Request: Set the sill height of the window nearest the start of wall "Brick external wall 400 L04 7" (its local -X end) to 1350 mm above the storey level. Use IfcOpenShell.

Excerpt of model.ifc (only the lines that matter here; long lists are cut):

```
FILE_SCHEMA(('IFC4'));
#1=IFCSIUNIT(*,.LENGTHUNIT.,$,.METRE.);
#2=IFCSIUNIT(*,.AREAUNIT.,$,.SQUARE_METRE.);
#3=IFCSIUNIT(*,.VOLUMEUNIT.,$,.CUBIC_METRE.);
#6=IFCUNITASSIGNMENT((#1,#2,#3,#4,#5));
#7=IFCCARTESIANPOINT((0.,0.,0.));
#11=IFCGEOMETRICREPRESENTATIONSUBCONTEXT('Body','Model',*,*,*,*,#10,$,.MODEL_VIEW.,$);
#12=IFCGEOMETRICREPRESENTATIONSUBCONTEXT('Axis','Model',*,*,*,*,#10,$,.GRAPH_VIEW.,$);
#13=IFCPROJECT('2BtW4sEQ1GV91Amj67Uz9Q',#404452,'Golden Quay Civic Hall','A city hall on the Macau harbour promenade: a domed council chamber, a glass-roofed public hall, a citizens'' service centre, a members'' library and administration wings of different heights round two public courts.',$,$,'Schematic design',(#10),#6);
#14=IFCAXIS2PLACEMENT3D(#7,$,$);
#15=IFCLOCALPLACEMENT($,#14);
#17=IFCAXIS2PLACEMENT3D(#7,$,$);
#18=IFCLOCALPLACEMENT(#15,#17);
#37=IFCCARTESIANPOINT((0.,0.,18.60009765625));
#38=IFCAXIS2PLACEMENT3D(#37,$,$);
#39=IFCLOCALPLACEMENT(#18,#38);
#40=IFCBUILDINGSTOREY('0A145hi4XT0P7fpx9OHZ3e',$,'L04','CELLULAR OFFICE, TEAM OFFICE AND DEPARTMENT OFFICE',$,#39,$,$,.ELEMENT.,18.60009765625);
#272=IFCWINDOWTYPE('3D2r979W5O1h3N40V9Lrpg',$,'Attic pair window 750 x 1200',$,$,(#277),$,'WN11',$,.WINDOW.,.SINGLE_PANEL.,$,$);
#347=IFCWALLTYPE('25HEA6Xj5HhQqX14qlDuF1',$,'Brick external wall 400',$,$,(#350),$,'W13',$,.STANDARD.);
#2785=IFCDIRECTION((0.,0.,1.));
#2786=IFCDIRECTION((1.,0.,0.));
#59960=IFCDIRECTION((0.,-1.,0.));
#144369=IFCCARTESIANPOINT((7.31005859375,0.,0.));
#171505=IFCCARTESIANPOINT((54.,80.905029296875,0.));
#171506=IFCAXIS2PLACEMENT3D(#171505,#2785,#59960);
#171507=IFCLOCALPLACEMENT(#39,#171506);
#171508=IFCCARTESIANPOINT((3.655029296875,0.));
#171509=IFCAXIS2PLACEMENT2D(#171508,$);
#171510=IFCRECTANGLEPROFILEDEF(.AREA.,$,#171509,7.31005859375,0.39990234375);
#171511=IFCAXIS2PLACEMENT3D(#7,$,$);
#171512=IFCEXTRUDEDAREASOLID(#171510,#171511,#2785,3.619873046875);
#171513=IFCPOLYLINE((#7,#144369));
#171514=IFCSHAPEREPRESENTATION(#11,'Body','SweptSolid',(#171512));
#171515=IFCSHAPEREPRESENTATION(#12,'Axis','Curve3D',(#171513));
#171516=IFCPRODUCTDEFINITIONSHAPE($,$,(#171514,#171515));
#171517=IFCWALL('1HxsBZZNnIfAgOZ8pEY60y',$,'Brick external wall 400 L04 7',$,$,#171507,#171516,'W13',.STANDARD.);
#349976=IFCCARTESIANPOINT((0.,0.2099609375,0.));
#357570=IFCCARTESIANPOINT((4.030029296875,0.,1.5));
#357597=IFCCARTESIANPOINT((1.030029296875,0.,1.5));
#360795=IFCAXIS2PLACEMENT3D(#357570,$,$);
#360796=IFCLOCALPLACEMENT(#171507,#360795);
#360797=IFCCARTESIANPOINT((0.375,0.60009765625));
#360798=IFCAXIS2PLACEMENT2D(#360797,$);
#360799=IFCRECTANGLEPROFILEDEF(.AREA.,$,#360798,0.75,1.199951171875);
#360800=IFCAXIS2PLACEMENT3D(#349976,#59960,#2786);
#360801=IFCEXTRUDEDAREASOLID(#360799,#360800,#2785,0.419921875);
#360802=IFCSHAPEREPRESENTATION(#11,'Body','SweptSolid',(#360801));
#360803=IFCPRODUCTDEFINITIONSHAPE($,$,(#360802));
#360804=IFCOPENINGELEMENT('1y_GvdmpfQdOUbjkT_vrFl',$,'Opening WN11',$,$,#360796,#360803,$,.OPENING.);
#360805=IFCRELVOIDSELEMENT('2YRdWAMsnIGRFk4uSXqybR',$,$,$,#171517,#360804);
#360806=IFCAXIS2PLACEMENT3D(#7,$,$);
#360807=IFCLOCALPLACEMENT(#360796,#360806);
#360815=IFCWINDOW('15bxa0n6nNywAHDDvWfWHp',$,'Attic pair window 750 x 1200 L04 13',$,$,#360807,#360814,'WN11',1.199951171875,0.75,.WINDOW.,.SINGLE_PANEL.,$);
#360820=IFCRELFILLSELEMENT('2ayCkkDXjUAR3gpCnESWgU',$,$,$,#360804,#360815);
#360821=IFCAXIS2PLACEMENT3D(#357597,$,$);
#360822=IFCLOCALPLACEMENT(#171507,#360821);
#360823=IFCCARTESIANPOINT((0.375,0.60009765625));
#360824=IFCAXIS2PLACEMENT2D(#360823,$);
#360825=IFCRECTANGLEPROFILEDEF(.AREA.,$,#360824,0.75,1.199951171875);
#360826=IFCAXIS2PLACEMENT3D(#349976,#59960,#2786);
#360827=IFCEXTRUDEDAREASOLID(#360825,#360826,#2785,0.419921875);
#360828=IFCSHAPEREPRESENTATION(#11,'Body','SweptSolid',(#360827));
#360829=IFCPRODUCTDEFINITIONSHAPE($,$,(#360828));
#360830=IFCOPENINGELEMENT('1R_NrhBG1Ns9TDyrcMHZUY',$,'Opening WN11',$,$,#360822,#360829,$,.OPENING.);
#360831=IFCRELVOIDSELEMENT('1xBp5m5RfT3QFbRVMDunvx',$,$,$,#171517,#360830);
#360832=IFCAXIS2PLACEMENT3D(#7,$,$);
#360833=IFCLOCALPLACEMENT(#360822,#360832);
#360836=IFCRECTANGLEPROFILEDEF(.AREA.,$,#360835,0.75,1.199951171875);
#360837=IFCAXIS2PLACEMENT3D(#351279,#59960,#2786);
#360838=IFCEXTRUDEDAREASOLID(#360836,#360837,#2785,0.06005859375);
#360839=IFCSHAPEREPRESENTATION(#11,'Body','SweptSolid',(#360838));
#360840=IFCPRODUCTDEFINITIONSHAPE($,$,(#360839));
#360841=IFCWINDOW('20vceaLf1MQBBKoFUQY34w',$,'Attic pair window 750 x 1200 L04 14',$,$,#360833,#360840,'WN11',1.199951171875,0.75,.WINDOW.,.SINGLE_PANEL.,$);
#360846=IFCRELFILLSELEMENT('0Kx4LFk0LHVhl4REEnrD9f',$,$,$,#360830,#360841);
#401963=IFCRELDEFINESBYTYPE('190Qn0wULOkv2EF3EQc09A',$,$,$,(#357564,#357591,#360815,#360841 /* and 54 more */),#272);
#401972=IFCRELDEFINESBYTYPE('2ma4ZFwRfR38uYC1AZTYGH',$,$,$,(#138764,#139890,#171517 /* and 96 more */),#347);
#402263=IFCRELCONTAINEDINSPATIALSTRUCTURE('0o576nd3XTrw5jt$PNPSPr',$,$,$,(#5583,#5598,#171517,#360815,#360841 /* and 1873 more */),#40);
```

```python
import numpy as np
import ifcopenshell
import ifcopenshell.api.geometry
import ifcopenshell.geom
import ifcopenshell.util.element
import ifcopenshell.util.placement
import ifcopenshell.util.shape
import ifcopenshell.util.unit

model = ifcopenshell.open("model.ifc")
unit_scale = ifcopenshell.util.unit.calculate_unit_scale(model)

window = model.by_id(360841)
opening = window.FillsVoids[0].RelatingOpeningElement
storey = ifcopenshell.util.element.get_container(window, ifc_class="IfcBuildingStorey")
level = ifcopenshell.util.placement.get_local_placement(storey.ObjectPlacement)[2, 3]

# The opening's origin need not be at the sill, so measure its lowest point.
shape = ifcopenshell.geom.create_shape(ifcopenshell.geom.settings(), opening)
bottom = ifcopenshell.util.shape.get_shape_bottom_elevation(shape, shape.geometry) / unit_scale
dz = level + 1.35 / unit_scale - bottom

shift = np.array([0.0, 0.0, dz])
# The window is placed relative to its opening, so it follows when the opening moves.
matrix = ifcopenshell.util.placement.get_local_placement(opening.ObjectPlacement)
matrix[:3, 3] += shift
ifcopenshell.api.geometry.edit_object_placement(
    model, product=opening, matrix=matrix, is_si=False, should_transform_children=True
)

print(f"moved by {dz * unit_scale:+.3f} m")

model.write("model_edited.ifc")
```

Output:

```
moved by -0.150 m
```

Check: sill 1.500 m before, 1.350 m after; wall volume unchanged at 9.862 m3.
